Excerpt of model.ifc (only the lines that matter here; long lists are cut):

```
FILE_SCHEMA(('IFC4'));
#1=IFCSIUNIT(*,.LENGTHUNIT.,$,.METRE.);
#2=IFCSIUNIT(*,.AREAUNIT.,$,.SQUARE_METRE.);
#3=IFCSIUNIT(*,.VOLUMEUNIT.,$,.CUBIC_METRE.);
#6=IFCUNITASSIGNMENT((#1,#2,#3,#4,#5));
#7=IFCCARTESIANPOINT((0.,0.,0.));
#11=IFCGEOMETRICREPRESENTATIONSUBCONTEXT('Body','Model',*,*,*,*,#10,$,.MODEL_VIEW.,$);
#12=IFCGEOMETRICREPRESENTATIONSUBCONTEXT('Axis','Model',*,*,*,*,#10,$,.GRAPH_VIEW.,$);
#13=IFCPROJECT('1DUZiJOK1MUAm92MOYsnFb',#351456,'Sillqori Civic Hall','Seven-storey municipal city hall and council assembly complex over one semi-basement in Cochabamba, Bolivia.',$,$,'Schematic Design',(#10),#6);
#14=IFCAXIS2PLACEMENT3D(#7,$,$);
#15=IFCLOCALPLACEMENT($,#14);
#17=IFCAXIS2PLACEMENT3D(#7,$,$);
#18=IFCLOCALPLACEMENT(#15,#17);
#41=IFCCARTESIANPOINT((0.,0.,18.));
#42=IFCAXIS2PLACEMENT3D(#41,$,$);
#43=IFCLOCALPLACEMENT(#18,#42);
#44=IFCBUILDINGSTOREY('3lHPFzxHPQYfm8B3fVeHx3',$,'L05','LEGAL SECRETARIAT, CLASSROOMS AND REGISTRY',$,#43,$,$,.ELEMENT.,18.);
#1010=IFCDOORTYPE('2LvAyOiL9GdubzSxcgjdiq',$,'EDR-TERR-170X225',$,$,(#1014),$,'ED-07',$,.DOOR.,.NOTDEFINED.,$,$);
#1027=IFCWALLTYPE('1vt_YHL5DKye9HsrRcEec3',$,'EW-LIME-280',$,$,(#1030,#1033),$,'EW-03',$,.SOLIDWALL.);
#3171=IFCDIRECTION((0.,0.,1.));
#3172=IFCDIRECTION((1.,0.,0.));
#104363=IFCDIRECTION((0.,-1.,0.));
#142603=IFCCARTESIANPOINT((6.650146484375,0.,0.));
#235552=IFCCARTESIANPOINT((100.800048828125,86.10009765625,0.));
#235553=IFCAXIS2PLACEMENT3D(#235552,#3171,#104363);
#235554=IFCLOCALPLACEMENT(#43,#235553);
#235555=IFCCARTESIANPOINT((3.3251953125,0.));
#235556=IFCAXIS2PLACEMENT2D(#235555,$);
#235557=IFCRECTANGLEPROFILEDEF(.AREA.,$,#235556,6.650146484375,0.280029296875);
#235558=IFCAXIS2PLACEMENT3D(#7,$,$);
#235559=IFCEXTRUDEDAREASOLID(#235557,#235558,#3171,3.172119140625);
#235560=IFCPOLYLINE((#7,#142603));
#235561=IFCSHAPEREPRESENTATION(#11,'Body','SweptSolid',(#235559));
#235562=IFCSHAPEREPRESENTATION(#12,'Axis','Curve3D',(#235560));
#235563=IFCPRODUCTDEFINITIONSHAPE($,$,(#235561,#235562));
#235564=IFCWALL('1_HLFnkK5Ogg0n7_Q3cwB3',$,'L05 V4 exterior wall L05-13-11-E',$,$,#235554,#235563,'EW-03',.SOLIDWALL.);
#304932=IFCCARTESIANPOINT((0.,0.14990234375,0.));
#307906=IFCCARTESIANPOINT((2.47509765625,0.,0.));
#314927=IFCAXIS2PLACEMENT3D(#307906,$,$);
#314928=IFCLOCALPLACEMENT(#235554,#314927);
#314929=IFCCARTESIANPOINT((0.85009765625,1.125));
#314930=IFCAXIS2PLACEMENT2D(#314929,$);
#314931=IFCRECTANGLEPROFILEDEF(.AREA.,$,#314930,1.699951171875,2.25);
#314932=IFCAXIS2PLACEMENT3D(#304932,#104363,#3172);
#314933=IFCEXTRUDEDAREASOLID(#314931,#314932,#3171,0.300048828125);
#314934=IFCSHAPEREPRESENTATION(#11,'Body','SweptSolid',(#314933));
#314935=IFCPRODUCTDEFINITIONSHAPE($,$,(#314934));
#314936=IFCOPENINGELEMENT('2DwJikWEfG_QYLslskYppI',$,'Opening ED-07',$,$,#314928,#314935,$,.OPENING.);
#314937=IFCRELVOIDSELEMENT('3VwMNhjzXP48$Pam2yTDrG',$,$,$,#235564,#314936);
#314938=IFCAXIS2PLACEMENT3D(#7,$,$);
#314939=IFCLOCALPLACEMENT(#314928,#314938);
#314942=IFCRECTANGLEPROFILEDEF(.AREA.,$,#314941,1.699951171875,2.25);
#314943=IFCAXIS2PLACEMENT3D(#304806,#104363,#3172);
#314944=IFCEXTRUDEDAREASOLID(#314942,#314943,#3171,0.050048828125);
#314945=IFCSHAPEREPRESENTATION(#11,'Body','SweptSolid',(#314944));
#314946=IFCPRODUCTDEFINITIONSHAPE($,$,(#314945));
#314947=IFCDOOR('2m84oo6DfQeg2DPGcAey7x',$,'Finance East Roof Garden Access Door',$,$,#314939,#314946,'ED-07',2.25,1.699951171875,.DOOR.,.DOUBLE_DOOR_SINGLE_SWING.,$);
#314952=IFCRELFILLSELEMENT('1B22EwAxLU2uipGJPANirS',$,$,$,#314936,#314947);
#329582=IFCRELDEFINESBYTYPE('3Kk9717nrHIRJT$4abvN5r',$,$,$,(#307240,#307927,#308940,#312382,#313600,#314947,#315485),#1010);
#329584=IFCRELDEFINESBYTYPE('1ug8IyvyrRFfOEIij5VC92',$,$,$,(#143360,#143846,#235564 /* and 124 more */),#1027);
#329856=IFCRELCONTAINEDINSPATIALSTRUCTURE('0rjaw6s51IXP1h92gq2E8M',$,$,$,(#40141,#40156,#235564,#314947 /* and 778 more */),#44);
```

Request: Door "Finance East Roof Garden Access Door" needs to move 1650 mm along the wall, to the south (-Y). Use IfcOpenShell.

```python
import ifcopenshell
import ifcopenshell.api.geometry
import ifcopenshell.util.placement
import ifcopenshell.util.unit

model = ifcopenshell.open("model.ifc")
unit_scale = ifcopenshell.util.unit.calculate_unit_scale(model)

door = model.by_id(314947)
opening = door.FillsVoids[0].RelatingOpeningElement
wall = opening.VoidsElements[0].RelatingBuildingElement

wall_matrix = ifcopenshell.util.placement.get_local_placement(wall.ObjectPlacement)
shift = wall_matrix[:3, 0] * 1.65 / unit_scale
before = ifcopenshell.util.placement.get_local_placement(door.ObjectPlacement)[:3, 3].copy()

# The door is placed relative to its opening, so it follows when the opening moves.
matrix = ifcopenshell.util.placement.get_local_placement(opening.ObjectPlacement)
matrix[:3, 3] += shift
ifcopenshell.api.geometry.edit_object_placement(
    model, product=opening, matrix=matrix, is_si=False, should_transform_children=True
)

after = ifcopenshell.util.placement.get_local_placement(door.ObjectPlacement)[:3, 3]
print("door moved by", (after - before).round(3) + 0.0)

model.write("model_edited.ifc")
```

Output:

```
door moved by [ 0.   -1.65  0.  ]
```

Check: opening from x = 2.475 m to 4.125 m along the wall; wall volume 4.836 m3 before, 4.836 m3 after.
